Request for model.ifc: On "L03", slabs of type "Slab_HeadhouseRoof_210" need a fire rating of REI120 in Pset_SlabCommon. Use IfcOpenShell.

First a look at what the model holds.

```python
import ifcopenshell
import ifcopenshell.util.element

model = ifcopenshell.open("model.ifc")
print(model.schema)
storey = next(s for s in model.by_type("IfcBuildingStorey") if s.Name == "L03")
slabs = [e for e in ifcopenshell.util.element.get_decomposition(storey) if e.is_a("IfcSlab")]
seen = {}
for e in slabs:
    element_type = ifcopenshell.util.element.get_type(e)
    key = (element_type.Name if element_type != e and element_type else None, ifcopenshell.util.element.get_pset(e, "Pset_SlabCommon", "FireRating"))
    seen[key] = seen.get(key, 0) + 1
for (name, value), count in sorted(seen.items(), key=str):
    print(count, "x", name, "|", value)
```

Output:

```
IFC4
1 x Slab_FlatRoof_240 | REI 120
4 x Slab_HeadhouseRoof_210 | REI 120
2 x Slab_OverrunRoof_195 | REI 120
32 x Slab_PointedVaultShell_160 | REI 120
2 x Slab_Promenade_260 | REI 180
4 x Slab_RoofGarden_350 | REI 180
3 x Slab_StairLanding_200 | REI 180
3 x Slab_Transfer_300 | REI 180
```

```python
import ifcopenshell
import ifcopenshell.api.pset
import ifcopenshell.util.element

model = ifcopenshell.open("model.ifc")

storey = next(s for s in model.by_type("IfcBuildingStorey") if s.Name == "L03")
slabs = [e for e in ifcopenshell.util.element.get_decomposition(storey) if e.is_a("IfcSlab")]

count = 0
for e in slabs:
    element_type = ifcopenshell.util.element.get_type(e)
    if element_type in (None, e) or element_type.Name != "Slab_HeadhouseRoof_210":
        continue
    # add_pset returns the element's existing set when there is one.
    pset = ifcopenshell.api.pset.add_pset(model, product=e, name="Pset_SlabCommon")
    ifcopenshell.api.pset.edit_pset(model, pset=pset, properties={"FireRating": "REI120"})
    count += 1

print(count, "slabs updated")

model.write("model_v2.ifc")
```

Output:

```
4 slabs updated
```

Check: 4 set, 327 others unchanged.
